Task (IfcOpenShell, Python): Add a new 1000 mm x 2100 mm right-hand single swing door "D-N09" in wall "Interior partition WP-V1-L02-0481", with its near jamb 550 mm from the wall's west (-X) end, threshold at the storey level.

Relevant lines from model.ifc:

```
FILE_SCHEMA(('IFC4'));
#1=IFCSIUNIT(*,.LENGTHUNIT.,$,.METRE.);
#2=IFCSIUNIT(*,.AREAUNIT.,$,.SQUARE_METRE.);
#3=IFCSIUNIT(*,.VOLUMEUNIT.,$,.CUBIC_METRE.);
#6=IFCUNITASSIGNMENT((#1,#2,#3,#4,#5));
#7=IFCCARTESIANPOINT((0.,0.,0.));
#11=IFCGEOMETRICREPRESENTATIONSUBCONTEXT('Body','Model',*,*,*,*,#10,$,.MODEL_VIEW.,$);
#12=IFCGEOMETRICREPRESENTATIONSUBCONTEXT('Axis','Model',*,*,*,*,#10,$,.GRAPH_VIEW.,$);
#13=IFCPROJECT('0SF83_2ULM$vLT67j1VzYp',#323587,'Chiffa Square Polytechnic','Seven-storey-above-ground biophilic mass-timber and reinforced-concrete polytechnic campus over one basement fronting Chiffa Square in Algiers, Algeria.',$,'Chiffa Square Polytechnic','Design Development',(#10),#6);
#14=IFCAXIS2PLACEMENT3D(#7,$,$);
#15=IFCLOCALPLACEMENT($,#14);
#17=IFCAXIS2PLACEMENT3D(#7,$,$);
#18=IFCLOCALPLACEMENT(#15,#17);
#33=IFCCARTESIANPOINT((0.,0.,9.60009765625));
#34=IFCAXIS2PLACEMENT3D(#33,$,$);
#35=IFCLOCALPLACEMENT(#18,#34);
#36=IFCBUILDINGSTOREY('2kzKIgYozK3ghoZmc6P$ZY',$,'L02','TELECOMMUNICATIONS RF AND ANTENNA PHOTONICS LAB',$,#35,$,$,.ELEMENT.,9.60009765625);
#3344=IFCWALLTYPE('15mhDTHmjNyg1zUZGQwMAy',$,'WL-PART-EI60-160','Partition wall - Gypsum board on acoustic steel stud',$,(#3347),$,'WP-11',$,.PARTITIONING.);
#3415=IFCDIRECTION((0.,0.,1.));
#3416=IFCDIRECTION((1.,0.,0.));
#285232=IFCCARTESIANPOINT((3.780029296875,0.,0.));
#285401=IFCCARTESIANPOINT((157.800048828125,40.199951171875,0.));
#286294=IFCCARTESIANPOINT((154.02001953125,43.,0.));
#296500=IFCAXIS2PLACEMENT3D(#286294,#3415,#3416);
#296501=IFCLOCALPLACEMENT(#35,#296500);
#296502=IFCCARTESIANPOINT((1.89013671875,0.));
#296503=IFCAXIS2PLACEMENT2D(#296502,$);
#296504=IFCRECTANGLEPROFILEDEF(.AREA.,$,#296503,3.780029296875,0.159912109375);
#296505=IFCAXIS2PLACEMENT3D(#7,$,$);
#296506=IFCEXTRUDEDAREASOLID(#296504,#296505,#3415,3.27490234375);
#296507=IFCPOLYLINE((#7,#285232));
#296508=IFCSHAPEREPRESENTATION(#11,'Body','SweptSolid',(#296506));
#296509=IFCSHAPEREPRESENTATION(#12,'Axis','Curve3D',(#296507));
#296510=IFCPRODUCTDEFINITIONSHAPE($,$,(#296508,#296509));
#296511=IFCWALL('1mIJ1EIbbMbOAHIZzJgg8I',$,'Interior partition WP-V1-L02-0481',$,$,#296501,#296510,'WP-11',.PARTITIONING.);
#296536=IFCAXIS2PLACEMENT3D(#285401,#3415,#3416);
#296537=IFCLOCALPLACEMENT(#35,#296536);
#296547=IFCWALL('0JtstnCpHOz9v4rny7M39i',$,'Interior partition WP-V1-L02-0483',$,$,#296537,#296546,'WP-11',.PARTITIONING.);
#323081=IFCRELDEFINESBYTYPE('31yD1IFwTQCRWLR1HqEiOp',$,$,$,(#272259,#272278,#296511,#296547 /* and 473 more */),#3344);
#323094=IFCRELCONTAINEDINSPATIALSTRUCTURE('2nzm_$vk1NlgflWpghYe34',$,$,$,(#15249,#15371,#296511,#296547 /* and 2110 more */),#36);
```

```python
import numpy as np
import ifcopenshell
import ifcopenshell.api.feature
import ifcopenshell.api.geometry
import ifcopenshell.api.root
import ifcopenshell.api.spatial
import ifcopenshell.geom
import ifcopenshell.util.element
import ifcopenshell.util.placement
import ifcopenshell.util.representation
import ifcopenshell.util.shape
import ifcopenshell.util.unit

model = ifcopenshell.open("model.ifc")
unit_scale = ifcopenshell.util.unit.calculate_unit_scale(model)
settings = ifcopenshell.geom.settings()


def volume(element):
    """Net volume in cubic metres, openings subtracted."""
    shape = ifcopenshell.geom.create_shape(settings, element)
    return ifcopenshell.util.shape.get_volume(shape.geometry)


wall = model.by_guid("1mIJ1EIbbMbOAHIZzJgg8I")
storey = ifcopenshell.util.element.get_container(wall, ifc_class="IfcBuildingStorey")
context = ifcopenshell.util.representation.get_context(model, "Model", "Body", "MODEL_VIEW")
before = volume(wall)

width, height, from_end, sill = 1, 2.1, 0.55, 0.0  # metres

# The wall runs along its own X axis, and the end named is its -X end.
wall_shape = ifcopenshell.geom.create_shape(settings, wall)
x, y, z = ifcopenshell.util.shape.get_vertices(wall_shape.geometry).T
start = x.min() + from_end
face, thickness = float(y.min()), float(y.max() - y.min())
wall_matrix = ifcopenshell.util.placement.get_local_placement(wall.ObjectPlacement)
level = ifcopenshell.util.placement.get_local_placement(storey.ObjectPlacement)[2, 3]


def in_wall(x, y):
    """Placement at x, y metres in the wall's axes, at sill height."""
    matrix = wall_matrix.copy()
    matrix[:, 3] = wall_matrix @ np.array([x / unit_scale, y / unit_scale, 0.0, 1.0])
    matrix[2, 3] = level + sill / unit_scale
    return matrix


# Opening: a box that overshoots both wall faces by 50 mm.
opening = ifcopenshell.api.root.create_entity(model, ifc_class="IfcOpeningElement", predefined_type="OPENING")
box = ifcopenshell.api.geometry.add_wall_representation(
    model, context=context, length=width, height=height, thickness=thickness + 0.1
)
ifcopenshell.api.geometry.assign_representation(model, product=opening, representation=box)
ifcopenshell.api.geometry.edit_object_placement(model, product=opening, matrix=in_wall(start, face - 0.05), is_si=False)
ifcopenshell.api.feature.add_feature(model, feature=opening, element=wall)

door = ifcopenshell.api.root.create_entity(model, ifc_class="IfcDoor", name="D-N09", predefined_type="DOOR")
door.OverallWidth, door.OverallHeight = width / unit_scale, height / unit_scale
door.OperationType = "SINGLE_SWING_RIGHT"
body = ifcopenshell.api.geometry.add_door_representation(
    model,
    context=context,
    overall_width=door.OverallWidth,
    overall_height=door.OverallHeight,
    operation_type="SINGLE_SWING_RIGHT",
    lining_properties={"LiningDepth": thickness / unit_scale, "ThresholdDepth": thickness / unit_scale},
)
ifcopenshell.api.geometry.assign_representation(model, product=door, representation=body)
ifcopenshell.api.spatial.assign_container(model, products=[door], relating_structure=storey)
ifcopenshell.api.feature.add_filling(model, opening=opening, element=door)

# The lining spans the wall, so the door starts at the wall face.
ifcopenshell.api.geometry.edit_object_placement(model, product=door, matrix=in_wall(start, face), is_si=False)

after = volume(wall)

print(f"wall volume {before:.3f} -> {after:.3f} m3")

model.write("model-out.ifc")
```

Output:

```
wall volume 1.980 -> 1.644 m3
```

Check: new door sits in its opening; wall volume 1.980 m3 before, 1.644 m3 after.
